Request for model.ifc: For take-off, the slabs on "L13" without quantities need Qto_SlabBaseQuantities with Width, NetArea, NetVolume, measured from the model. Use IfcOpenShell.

First a look at what the model holds.

```python
import ifcopenshell
import ifcopenshell.util.element
import ifcopenshell.util.unit

model = ifcopenshell.open("model.ifc")
print(model.schema)
for unit_type in ("LENGTHUNIT", "AREAUNIT", "VOLUMEUNIT"):
    print(unit_type, ifcopenshell.util.unit.calculate_unit_scale(model, unit_type))
storey = next(s for s in model.by_type("IfcBuildingStorey") if s.Name == "L13")
slabs = [e for e in ifcopenshell.util.element.get_decomposition(storey) if e.is_a("IfcSlab")]
for e in sorted(slabs, key=lambda e: e.id()):
    print(e.id(), e.is_a(), e.Name, list(ifcopenshell.util.element.get_psets(e, qtos_only=True)), sep=" | ")
```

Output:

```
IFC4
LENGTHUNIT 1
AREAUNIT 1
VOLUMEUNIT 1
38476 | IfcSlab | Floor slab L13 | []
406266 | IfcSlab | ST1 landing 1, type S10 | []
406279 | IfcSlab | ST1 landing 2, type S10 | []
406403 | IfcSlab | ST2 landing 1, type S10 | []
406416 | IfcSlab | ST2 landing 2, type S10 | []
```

```python
import ifcopenshell
import ifcopenshell.api.pset
import ifcopenshell.geom
import ifcopenshell.util.element
import ifcopenshell.util.shape
import ifcopenshell.util.unit

model = ifcopenshell.open("model.ifc")
unit_scale = ifcopenshell.util.unit.calculate_unit_scale(model)
area_scale = ifcopenshell.util.unit.calculate_unit_scale(model, "AREAUNIT")
volume_scale = ifcopenshell.util.unit.calculate_unit_scale(model, "VOLUMEUNIT")
settings = ifcopenshell.geom.settings()

storey = next(s for s in model.by_type("IfcBuildingStorey") if s.Name == "L13")
slabs = [e for e in ifcopenshell.util.element.get_decomposition(storey) if e.is_a("IfcSlab")]

for e in sorted(slabs, key=lambda e: e.id()):
    if ifcopenshell.util.element.get_psets(e, qtos_only=True, should_inherit=False):
        continue
    # Geometry comes back in metres, in the element's own axes.
    shape = ifcopenshell.geom.create_shape(settings, e)
    values = {
        "Width": ifcopenshell.util.shape.get_z(shape.geometry) / unit_scale,
        "NetArea": ifcopenshell.util.shape.get_footprint_area(shape.geometry) / area_scale,
        "NetVolume": ifcopenshell.util.shape.get_volume(shape.geometry) / volume_scale,
    }
    qto = ifcopenshell.api.pset.add_qto(model, product=e, name="Qto_SlabBaseQuantities")
    ifcopenshell.api.pset.edit_qto(model, qto=qto, properties=values)
    print(e.id(), {k: round(v, 3) for k, v in values.items()})

model.write("model-out.ifc")
```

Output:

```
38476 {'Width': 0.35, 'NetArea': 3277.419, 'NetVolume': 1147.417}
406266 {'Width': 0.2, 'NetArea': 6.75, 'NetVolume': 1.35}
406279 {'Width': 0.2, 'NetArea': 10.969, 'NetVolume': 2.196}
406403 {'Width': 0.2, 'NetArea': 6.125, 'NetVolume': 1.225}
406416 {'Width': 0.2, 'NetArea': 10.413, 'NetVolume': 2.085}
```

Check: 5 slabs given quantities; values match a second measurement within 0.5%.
